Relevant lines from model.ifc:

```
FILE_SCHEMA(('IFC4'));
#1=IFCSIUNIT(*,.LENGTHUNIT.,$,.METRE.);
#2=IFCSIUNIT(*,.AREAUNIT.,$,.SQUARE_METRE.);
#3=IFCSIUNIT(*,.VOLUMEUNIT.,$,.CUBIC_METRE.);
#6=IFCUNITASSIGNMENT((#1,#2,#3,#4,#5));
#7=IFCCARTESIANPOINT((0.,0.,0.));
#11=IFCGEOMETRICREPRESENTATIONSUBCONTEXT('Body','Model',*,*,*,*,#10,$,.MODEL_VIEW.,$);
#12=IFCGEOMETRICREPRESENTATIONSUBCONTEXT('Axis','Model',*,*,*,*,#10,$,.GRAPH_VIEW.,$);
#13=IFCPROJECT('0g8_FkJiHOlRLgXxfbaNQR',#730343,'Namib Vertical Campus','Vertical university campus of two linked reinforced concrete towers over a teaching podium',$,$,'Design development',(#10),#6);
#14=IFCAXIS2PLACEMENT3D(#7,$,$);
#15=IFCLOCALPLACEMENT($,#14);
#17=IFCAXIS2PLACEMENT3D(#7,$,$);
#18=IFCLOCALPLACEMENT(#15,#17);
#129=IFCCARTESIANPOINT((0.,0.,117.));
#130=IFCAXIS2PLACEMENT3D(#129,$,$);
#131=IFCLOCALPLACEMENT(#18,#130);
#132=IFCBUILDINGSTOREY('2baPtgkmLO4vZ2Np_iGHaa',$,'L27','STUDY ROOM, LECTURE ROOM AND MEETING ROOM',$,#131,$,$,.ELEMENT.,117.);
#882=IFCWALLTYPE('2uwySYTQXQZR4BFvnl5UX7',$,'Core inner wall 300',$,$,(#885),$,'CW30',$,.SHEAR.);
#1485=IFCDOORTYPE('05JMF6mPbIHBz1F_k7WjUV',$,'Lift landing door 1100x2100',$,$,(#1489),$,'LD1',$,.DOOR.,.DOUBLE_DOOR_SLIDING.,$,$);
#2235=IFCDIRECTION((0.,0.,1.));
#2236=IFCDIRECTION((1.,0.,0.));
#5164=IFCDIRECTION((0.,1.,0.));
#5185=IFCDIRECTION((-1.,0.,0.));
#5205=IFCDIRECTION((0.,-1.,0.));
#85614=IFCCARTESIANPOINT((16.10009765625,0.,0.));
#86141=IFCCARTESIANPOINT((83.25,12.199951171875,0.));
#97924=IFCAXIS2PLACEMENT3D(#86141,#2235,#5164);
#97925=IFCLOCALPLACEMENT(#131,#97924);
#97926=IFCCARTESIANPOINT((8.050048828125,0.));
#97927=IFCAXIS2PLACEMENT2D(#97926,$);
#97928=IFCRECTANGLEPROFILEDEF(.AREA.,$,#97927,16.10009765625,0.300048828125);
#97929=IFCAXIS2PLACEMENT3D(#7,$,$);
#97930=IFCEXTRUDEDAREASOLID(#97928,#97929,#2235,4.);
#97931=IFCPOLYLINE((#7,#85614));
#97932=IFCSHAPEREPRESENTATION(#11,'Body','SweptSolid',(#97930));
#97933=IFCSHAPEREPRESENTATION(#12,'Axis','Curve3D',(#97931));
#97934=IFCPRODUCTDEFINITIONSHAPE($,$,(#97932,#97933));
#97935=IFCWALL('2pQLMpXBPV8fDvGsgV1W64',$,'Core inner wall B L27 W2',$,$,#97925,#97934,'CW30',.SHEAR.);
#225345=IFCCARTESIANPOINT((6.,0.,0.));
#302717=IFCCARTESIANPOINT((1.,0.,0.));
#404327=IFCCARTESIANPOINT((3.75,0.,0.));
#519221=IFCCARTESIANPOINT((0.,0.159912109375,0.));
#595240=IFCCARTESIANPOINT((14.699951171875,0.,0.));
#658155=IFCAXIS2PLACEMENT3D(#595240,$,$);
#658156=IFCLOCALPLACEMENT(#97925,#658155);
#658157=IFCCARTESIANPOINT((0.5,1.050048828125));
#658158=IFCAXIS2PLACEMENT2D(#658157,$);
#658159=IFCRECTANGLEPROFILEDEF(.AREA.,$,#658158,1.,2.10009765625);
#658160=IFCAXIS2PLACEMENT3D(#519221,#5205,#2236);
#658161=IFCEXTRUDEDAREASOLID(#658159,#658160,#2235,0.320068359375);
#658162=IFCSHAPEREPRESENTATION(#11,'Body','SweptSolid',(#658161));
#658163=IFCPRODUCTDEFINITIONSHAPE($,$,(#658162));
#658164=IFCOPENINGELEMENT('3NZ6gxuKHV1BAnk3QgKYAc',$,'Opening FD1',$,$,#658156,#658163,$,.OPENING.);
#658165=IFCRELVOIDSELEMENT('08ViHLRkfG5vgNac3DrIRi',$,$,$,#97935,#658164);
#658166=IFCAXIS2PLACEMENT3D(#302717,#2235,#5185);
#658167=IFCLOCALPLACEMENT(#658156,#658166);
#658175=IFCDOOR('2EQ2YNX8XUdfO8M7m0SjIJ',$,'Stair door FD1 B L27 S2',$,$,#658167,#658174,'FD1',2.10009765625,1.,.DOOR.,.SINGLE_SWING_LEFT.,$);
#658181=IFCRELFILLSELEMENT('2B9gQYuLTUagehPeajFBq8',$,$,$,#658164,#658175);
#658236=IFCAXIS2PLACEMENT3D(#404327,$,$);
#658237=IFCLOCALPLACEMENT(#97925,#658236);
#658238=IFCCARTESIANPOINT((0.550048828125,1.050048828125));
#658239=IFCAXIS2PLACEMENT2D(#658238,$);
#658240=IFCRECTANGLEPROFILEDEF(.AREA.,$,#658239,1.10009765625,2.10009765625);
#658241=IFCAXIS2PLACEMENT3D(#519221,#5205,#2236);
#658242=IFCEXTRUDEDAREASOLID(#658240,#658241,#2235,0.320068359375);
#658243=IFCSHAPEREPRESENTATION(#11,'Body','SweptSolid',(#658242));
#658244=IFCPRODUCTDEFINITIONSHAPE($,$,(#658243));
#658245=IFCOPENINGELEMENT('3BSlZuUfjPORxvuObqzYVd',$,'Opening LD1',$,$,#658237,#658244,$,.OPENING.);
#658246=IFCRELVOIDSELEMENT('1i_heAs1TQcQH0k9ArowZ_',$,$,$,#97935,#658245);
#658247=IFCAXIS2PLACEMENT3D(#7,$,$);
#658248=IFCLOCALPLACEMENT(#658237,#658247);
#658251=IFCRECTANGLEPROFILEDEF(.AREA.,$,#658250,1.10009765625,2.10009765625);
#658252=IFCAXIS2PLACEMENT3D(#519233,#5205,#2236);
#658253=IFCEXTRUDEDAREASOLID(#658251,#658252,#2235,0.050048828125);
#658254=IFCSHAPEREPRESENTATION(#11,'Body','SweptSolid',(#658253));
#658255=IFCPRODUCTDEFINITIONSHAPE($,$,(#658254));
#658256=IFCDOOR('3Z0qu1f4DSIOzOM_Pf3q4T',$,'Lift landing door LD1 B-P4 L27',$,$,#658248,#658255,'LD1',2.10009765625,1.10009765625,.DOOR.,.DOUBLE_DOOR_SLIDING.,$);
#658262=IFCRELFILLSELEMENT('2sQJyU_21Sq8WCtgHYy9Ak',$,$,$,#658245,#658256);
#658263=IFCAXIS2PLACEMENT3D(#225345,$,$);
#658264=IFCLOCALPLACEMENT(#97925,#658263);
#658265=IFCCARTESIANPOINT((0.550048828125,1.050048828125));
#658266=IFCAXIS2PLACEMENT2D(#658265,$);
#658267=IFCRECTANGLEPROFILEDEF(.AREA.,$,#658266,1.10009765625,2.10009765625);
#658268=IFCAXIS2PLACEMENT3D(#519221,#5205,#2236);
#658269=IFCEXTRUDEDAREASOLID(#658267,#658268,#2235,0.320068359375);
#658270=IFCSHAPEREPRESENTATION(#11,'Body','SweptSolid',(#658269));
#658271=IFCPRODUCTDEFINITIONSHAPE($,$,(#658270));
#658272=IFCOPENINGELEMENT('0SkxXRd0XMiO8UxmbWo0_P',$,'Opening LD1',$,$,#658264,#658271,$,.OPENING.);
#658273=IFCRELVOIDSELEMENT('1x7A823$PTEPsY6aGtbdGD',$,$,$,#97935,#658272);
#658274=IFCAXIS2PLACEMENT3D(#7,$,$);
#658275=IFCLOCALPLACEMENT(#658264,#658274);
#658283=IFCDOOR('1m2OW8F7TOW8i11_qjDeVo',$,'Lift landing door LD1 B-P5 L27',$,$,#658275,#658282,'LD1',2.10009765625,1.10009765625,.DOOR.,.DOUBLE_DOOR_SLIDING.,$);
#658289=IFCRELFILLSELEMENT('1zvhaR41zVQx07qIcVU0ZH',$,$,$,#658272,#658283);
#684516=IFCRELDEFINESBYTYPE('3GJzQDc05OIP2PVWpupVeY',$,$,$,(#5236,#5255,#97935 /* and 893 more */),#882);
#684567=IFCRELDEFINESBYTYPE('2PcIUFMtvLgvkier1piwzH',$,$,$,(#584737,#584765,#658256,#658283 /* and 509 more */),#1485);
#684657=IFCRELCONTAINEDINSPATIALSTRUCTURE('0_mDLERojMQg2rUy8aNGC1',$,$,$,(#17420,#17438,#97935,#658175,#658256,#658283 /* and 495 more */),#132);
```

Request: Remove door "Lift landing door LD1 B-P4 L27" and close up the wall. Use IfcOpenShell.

```python
import ifcopenshell
import ifcopenshell.api.feature
import ifcopenshell.api.root
import ifcopenshell.geom
import ifcopenshell.util.shape

model = ifcopenshell.open("model.ifc")
settings = ifcopenshell.geom.settings()


def volume(element):
    """Net volume in cubic metres, openings subtracted."""
    shape = ifcopenshell.geom.create_shape(settings, element)
    return ifcopenshell.util.shape.get_volume(shape.geometry)


door = model.by_guid("3Z0qu1f4DSIOzOM_Pf3q4T")
opening = door.FillsVoids[0].RelatingOpeningElement
wall = opening.VoidsElements[0].RelatingBuildingElement
before = volume(wall)

ifcopenshell.api.root.remove_product(model, product=door)
ifcopenshell.api.feature.remove_feature(model, feature=opening)

after = volume(wall)

print(f"wall volume {before:.3f} -> {after:.3f} m3")

model.write("model_edited.ifc")
```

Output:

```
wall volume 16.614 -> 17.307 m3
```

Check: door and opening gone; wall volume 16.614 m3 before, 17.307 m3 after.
